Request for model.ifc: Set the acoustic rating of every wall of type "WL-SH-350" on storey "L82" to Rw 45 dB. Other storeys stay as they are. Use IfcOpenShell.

First a look at what the model holds.

```python
import ifcopenshell
import ifcopenshell.util.element

model = ifcopenshell.open("model.ifc")
print(model.schema)
storey = next(s for s in model.by_type("IfcBuildingStorey") if s.Name == "L82")
walls = [e for e in ifcopenshell.util.element.get_decomposition(storey) if e.is_a("IfcWall")]
seen = {}
for e in walls:
    element_type = ifcopenshell.util.element.get_type(e)
    key = (element_type.Name if element_type != e and element_type else None, ifcopenshell.util.element.get_pset(e, "Pset_WallCommon", "AcousticRating"))
    seen[key] = seen.get(key, 0) + 1
for (name, value), count in sorted(seen.items(), key=str):
    print(count, "x", name, "|", value)
```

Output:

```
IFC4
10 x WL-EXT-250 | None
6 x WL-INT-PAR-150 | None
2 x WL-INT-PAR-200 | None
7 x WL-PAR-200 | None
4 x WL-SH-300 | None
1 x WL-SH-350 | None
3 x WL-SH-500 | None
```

```python
import ifcopenshell
import ifcopenshell.api.pset
import ifcopenshell.util.element

model = ifcopenshell.open("model.ifc")

storey = next(s for s in model.by_type("IfcBuildingStorey") if s.Name == "L82")
walls = [e for e in ifcopenshell.util.element.get_decomposition(storey) if e.is_a("IfcWall")]

count = 0
for e in walls:
    element_type = ifcopenshell.util.element.get_type(e)
    if element_type in (None, e) or element_type.Name != "WL-SH-350":
        continue
    found = ifcopenshell.util.element.get_pset(e, "Pset_WallCommon", should_inherit=False)
    if found:
        pset = model.by_id(found["id"])
        if len(ifcopenshell.util.element.get_elements_by_pset(pset)) > 1:
            pset = ifcopenshell.api.pset.unshare_pset(model, products=[e], pset=pset)[0]
    else:
        pset = ifcopenshell.api.pset.add_pset(model, product=e, name="Pset_WallCommon")
    ifcopenshell.api.pset.edit_pset(model, pset=pset, properties={"AcousticRating": "Rw 45 dB"})
    count += 1

print(count, "walls updated")

model.write("model_edited.ifc")
```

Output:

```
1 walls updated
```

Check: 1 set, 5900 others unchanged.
